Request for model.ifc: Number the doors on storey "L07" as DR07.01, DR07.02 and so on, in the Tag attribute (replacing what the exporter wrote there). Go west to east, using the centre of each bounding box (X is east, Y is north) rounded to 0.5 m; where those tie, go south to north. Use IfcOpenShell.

First a look at what the model holds.

```python
import ifcopenshell
import ifcopenshell.util.element
import ifcopenshell.util.placement

model = ifcopenshell.open("model.ifc")
print(model.schema)
storey = next(s for s in model.by_type("IfcBuildingStorey") if s.Name == "L07")
doors = [e for e in ifcopenshell.util.element.get_decomposition(storey) if e.is_a("IfcDoor")]
for e in sorted(doors, key=lambda e: e.id()):
    origin = ifcopenshell.util.placement.get_local_placement(e.ObjectPlacement)[:3, 3]
    print(e.id(), e.Tag, e.Name, origin.round(2) + 0.0, sep=" | ")
```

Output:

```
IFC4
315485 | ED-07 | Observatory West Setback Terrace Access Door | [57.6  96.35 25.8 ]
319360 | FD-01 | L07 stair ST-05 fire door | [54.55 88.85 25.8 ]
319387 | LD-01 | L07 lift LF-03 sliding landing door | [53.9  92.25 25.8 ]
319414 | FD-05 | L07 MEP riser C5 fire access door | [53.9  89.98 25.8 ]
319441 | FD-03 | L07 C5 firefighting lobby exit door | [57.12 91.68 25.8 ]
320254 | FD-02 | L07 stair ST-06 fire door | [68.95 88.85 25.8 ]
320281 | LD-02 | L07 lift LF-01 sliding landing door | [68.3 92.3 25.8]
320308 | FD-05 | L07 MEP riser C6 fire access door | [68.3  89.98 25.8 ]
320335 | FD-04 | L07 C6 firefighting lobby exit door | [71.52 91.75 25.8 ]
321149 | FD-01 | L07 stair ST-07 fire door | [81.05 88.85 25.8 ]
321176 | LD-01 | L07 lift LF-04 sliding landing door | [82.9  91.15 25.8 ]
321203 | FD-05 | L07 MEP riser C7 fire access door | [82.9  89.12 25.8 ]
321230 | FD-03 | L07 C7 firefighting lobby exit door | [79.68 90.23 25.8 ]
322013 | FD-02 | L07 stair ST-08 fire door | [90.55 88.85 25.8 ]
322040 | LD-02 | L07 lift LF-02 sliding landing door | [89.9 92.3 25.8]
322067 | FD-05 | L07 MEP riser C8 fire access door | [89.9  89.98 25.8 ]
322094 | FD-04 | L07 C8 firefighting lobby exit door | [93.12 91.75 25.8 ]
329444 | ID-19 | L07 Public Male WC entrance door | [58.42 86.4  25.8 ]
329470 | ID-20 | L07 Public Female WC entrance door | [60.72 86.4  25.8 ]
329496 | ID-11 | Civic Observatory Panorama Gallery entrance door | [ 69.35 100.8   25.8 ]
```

```python
import ifcopenshell
import ifcopenshell.geom
import ifcopenshell.util.element
import ifcopenshell.util.shape

model = ifcopenshell.open("model.ifc")
settings = ifcopenshell.geom.settings()
settings.set("use-world-coords", True)


def centre(element):
    shape = ifcopenshell.geom.create_shape(settings, element)
    return ifcopenshell.util.shape.get_bbox_centroid(shape.geometry)


storey = next(s for s in model.by_type("IfcBuildingStorey") if s.Name == "L07")
doors = [e for e in ifcopenshell.util.element.get_decomposition(storey) if e.is_a("IfcDoor")]

# Insertion points can sit at a corner or the storey origin, so sort by the geometry (in metres).
centres = {e: centre(e) for e in doors}
doors.sort(key=lambda e: (round(centres[e][0] / 0.5), centres[e][1]))

for i, e in enumerate(doors, start=1):
    number = f"DR07.{i:02d}"
    e.Tag = number
    print(e.id(), number)

model.write("model_rev.ifc")
```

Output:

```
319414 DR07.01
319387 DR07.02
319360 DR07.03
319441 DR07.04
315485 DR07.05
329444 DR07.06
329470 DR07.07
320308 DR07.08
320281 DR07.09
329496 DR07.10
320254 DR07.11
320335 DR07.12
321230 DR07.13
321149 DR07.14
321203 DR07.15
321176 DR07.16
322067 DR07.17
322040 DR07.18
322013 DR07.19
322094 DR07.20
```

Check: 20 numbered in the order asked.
